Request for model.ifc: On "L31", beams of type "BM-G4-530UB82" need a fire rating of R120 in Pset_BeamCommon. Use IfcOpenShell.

First a look at what the model holds.

```python
import ifcopenshell
import ifcopenshell.util.element

model = ifcopenshell.open("model.ifc")
print(model.schema)
storey = next(s for s in model.by_type("IfcBuildingStorey") if s.Name == "L31")
beams = [e for e in ifcopenshell.util.element.get_decomposition(storey) if e.is_a("IfcBeam")]
seen = {}
for e in beams:
    element_type = ifcopenshell.util.element.get_type(e)
    key = (element_type.Name if element_type != e and element_type else None, ifcopenshell.util.element.get_pset(e, "Pset_BeamCommon", "FireRating"))
    seen[key] = seen.get(key, 0) + 1
for (name, value), count in sorted(seen.items(), key=str):
    print(count, "x", name, "|", value)
```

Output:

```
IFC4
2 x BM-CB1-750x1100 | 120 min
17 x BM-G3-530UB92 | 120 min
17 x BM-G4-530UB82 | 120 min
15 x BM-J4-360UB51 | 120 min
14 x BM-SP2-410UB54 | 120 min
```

```python
import ifcopenshell
import ifcopenshell.api.pset
import ifcopenshell.util.element

model = ifcopenshell.open("model.ifc")

storey = next(s for s in model.by_type("IfcBuildingStorey") if s.Name == "L31")
beams = [e for e in ifcopenshell.util.element.get_decomposition(storey) if e.is_a("IfcBeam")]

count = 0
for e in beams:
    element_type = ifcopenshell.util.element.get_type(e)
    if element_type in (None, e) or element_type.Name != "BM-G4-530UB82":
        continue
    # add_pset returns the element's existing set when there is one.
    pset = ifcopenshell.api.pset.add_pset(model, product=e, name="Pset_BeamCommon")
    ifcopenshell.api.pset.edit_pset(model, pset=pset, properties={"FireRating": "R120"})
    count += 1

print(count, "beams updated")

model.write("model-out.ifc")
```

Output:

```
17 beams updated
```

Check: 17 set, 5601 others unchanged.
